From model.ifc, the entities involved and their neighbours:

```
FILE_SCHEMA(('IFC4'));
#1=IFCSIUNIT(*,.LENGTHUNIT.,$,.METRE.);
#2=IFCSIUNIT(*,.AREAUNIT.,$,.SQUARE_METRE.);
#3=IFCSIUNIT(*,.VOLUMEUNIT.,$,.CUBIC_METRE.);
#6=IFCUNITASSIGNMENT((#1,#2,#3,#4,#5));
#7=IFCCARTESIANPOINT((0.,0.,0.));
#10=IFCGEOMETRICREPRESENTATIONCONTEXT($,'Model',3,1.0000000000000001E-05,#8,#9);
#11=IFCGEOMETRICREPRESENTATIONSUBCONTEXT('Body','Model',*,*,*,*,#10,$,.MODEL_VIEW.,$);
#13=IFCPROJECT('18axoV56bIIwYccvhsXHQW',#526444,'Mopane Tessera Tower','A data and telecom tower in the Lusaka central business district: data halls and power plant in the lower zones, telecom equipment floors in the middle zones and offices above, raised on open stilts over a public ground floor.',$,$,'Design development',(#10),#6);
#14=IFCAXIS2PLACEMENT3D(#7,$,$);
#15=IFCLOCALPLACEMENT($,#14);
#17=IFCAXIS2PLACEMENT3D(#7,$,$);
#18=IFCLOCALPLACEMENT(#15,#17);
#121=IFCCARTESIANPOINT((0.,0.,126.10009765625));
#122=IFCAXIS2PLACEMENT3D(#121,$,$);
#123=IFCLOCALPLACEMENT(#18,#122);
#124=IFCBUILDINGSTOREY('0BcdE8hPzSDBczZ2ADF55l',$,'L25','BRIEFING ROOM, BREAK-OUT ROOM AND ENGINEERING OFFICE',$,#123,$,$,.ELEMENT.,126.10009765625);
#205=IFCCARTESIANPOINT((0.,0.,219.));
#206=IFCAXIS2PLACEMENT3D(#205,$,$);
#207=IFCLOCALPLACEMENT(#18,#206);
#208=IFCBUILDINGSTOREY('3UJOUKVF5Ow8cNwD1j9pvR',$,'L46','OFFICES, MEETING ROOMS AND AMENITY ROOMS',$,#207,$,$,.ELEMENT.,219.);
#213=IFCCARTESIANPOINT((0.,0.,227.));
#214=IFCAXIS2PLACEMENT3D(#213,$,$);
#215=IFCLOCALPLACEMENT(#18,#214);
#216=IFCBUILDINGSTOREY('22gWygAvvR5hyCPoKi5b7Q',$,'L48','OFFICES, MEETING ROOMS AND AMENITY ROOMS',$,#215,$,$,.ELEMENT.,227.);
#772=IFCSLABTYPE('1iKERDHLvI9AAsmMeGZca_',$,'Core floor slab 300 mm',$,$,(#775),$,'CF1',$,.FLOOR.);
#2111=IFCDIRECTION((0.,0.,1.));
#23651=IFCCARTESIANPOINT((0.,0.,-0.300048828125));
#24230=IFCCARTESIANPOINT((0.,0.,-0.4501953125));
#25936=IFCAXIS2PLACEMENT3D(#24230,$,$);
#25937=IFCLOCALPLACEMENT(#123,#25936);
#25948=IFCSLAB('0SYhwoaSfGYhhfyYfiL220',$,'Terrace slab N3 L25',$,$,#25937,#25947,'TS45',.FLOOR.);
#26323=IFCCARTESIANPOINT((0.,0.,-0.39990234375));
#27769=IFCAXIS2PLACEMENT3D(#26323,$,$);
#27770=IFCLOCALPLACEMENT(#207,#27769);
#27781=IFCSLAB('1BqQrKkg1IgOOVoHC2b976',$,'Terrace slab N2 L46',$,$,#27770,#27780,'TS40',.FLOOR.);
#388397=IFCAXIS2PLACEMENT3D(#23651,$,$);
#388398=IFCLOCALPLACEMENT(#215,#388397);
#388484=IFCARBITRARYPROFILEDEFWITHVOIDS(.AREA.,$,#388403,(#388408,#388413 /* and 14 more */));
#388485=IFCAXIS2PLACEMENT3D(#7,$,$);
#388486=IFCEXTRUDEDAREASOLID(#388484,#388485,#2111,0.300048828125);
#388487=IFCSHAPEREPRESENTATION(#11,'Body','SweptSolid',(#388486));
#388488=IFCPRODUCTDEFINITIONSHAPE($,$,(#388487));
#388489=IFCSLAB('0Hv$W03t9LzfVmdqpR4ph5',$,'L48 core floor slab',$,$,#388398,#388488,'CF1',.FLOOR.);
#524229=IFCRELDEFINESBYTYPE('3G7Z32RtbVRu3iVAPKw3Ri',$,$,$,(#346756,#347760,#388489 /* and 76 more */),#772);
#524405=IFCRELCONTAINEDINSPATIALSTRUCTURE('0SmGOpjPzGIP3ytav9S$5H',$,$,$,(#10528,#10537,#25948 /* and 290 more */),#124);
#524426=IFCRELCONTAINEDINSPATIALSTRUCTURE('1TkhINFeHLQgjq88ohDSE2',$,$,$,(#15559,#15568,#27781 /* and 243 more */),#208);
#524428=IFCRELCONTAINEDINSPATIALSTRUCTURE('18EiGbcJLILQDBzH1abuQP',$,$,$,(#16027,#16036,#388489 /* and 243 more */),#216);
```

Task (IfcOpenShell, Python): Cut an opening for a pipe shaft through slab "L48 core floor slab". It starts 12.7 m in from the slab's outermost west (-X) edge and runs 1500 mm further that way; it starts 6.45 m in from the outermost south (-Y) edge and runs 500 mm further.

```python
import numpy as np
import ifcopenshell
import ifcopenshell.api.feature
import ifcopenshell.api.geometry
import ifcopenshell.api.root
import ifcopenshell.geom
import ifcopenshell.util.placement
import ifcopenshell.util.representation
import ifcopenshell.util.shape
import ifcopenshell.util.unit

model = ifcopenshell.open("model.ifc")
unit_scale = ifcopenshell.util.unit.calculate_unit_scale(model)
settings = ifcopenshell.geom.settings()


def volume(element):
    """Net volume in cubic metres, openings subtracted."""
    shape = ifcopenshell.geom.create_shape(settings, element)
    return ifcopenshell.util.shape.get_volume(shape.geometry)


slab = model.by_id(388489)
before = volume(slab)

# Extent in the slab's own axes, in metres. The edges named are its -X and -Y sides.
slab_shape = ifcopenshell.geom.create_shape(settings, slab)
vertices = ifcopenshell.util.shape.get_vertices(slab_shape.geometry)
x_min, y_min, bottom = vertices.min(axis=0)
top = vertices[:, 2].max()

opening = ifcopenshell.api.root.create_entity(model, ifc_class="IfcOpeningElement", name="Pipe shaft opening", predefined_type="OPENING")
context = ifcopenshell.util.representation.get_context(model, "Model", "Body", "MODEL_VIEW")
width, depth = 1.5, 0.5
outline = [(0.0, 0.0), (width, 0.0), (width, depth), (0.0, depth), (0.0, 0.0)]
# Overshoot both faces by 50 mm so the cut is clean.
shape = ifcopenshell.api.geometry.add_slab_representation(
    model, context=context, depth=top - bottom + 0.1, polyline=outline
)
ifcopenshell.api.geometry.assign_representation(model, product=opening, representation=shape)

matrix = ifcopenshell.util.placement.get_local_placement(slab.ObjectPlacement)
matrix[:, 3] = matrix @ np.append(np.array([x_min + 12.7, y_min + 6.45, bottom - 0.05]) / unit_scale, 1.0)
ifcopenshell.api.geometry.edit_object_placement(model, product=opening, matrix=matrix, is_si=False)
ifcopenshell.api.feature.add_feature(model, feature=opening, element=slab)

after = volume(slab)

print(f"slab volume {before:.3f} -> {after:.3f} m3")

model.write("model_rev.ifc")
```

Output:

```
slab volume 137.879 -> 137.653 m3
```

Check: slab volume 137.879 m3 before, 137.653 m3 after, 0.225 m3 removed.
